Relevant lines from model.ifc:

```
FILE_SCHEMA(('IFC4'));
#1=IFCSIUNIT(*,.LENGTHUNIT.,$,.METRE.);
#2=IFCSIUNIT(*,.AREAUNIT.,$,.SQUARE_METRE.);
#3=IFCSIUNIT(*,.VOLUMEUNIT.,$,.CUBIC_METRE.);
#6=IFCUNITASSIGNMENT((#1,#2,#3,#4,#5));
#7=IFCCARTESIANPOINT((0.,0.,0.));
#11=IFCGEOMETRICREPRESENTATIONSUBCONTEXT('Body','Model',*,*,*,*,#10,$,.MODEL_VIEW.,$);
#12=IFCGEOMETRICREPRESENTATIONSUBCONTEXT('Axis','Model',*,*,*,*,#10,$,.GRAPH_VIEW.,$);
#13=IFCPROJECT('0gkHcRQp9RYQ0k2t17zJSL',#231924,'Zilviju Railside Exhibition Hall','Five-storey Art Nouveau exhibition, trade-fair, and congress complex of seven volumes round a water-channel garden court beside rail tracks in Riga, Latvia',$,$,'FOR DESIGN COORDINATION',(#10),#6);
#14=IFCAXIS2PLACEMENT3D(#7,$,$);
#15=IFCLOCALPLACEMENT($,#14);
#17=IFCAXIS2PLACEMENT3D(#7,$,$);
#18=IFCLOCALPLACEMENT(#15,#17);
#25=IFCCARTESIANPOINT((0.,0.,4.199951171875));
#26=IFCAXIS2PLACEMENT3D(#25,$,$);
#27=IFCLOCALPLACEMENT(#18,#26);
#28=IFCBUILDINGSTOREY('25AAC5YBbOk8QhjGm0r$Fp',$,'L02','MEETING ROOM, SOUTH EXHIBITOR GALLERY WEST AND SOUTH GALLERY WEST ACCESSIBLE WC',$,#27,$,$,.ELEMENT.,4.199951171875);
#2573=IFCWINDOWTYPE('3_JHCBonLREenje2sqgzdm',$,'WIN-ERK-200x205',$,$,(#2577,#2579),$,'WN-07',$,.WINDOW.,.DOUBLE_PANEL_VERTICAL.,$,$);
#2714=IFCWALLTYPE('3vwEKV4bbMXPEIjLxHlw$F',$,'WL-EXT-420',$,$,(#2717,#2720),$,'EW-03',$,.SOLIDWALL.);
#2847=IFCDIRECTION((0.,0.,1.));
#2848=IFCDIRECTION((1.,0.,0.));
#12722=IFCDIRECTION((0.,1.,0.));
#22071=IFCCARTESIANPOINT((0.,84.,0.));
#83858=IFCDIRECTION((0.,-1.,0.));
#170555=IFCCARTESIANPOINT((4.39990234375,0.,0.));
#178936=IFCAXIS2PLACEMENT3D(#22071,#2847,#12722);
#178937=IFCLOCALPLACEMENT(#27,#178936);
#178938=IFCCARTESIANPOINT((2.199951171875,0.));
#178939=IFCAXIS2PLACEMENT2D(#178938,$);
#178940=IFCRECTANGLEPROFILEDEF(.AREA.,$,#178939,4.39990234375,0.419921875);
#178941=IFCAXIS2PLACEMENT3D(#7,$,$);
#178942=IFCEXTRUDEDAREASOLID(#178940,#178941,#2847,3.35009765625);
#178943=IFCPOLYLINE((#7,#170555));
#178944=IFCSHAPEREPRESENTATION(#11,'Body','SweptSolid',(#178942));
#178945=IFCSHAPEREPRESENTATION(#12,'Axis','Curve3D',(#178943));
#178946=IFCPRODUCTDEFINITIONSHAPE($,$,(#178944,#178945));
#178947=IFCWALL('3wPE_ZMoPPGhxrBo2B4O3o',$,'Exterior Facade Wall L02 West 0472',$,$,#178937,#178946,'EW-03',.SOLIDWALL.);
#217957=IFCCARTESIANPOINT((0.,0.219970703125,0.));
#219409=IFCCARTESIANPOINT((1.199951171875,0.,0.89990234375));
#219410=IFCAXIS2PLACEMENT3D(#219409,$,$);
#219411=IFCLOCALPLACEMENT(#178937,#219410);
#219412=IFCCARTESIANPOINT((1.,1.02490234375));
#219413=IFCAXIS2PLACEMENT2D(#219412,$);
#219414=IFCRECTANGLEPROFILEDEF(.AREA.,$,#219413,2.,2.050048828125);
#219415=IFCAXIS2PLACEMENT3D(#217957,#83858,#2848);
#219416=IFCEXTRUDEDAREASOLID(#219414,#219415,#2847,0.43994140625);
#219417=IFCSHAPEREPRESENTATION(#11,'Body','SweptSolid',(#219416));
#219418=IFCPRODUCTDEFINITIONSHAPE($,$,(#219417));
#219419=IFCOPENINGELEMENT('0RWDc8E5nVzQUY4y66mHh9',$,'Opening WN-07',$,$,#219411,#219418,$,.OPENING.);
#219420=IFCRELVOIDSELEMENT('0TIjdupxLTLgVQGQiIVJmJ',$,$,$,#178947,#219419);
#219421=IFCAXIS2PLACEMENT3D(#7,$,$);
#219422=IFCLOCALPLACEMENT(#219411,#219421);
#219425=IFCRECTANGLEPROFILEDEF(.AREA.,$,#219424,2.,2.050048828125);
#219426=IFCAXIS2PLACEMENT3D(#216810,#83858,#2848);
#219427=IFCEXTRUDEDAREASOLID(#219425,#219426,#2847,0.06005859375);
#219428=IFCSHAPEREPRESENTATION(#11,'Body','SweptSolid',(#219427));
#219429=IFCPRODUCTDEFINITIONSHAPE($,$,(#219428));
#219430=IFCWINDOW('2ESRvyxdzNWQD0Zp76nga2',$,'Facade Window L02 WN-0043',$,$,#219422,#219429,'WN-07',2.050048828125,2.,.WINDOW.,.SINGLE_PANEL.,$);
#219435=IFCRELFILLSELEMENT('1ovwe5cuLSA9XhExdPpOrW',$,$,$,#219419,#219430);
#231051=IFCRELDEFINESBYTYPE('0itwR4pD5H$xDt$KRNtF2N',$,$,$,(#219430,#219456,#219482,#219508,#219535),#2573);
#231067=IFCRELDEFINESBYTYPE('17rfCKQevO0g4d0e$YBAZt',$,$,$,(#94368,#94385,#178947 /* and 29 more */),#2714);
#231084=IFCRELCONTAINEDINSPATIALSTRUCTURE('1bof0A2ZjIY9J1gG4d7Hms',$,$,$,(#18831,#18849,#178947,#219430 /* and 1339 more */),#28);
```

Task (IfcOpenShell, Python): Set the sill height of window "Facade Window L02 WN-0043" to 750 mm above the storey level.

```python
import numpy as np
import ifcopenshell
import ifcopenshell.api.geometry
import ifcopenshell.geom
import ifcopenshell.util.element
import ifcopenshell.util.placement
import ifcopenshell.util.shape
import ifcopenshell.util.unit

model = ifcopenshell.open("model.ifc")
unit_scale = ifcopenshell.util.unit.calculate_unit_scale(model)

window = model.by_id(219430)
opening = window.FillsVoids[0].RelatingOpeningElement
storey = ifcopenshell.util.element.get_container(window, ifc_class="IfcBuildingStorey")
level = ifcopenshell.util.placement.get_local_placement(storey.ObjectPlacement)[2, 3]

# The opening's origin need not be at the sill, so measure its lowest point.
shape = ifcopenshell.geom.create_shape(ifcopenshell.geom.settings(), opening)
bottom = ifcopenshell.util.shape.get_shape_bottom_elevation(shape, shape.geometry) / unit_scale
dz = level + 0.75 - bottom

shift = np.array([0.0, 0.0, dz])
# The window is placed relative to its opening, so it follows when the opening moves.
matrix = ifcopenshell.util.placement.get_local_placement(opening.ObjectPlacement)
matrix[:3, 3] += shift
ifcopenshell.api.geometry.edit_object_placement(
    model, product=opening, matrix=matrix, is_si=False, should_transform_children=True
)

print(f"moved by {dz * unit_scale:+.3f} m")

model.write("model_edited.ifc")
```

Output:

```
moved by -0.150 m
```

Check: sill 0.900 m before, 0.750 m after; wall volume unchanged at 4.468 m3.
